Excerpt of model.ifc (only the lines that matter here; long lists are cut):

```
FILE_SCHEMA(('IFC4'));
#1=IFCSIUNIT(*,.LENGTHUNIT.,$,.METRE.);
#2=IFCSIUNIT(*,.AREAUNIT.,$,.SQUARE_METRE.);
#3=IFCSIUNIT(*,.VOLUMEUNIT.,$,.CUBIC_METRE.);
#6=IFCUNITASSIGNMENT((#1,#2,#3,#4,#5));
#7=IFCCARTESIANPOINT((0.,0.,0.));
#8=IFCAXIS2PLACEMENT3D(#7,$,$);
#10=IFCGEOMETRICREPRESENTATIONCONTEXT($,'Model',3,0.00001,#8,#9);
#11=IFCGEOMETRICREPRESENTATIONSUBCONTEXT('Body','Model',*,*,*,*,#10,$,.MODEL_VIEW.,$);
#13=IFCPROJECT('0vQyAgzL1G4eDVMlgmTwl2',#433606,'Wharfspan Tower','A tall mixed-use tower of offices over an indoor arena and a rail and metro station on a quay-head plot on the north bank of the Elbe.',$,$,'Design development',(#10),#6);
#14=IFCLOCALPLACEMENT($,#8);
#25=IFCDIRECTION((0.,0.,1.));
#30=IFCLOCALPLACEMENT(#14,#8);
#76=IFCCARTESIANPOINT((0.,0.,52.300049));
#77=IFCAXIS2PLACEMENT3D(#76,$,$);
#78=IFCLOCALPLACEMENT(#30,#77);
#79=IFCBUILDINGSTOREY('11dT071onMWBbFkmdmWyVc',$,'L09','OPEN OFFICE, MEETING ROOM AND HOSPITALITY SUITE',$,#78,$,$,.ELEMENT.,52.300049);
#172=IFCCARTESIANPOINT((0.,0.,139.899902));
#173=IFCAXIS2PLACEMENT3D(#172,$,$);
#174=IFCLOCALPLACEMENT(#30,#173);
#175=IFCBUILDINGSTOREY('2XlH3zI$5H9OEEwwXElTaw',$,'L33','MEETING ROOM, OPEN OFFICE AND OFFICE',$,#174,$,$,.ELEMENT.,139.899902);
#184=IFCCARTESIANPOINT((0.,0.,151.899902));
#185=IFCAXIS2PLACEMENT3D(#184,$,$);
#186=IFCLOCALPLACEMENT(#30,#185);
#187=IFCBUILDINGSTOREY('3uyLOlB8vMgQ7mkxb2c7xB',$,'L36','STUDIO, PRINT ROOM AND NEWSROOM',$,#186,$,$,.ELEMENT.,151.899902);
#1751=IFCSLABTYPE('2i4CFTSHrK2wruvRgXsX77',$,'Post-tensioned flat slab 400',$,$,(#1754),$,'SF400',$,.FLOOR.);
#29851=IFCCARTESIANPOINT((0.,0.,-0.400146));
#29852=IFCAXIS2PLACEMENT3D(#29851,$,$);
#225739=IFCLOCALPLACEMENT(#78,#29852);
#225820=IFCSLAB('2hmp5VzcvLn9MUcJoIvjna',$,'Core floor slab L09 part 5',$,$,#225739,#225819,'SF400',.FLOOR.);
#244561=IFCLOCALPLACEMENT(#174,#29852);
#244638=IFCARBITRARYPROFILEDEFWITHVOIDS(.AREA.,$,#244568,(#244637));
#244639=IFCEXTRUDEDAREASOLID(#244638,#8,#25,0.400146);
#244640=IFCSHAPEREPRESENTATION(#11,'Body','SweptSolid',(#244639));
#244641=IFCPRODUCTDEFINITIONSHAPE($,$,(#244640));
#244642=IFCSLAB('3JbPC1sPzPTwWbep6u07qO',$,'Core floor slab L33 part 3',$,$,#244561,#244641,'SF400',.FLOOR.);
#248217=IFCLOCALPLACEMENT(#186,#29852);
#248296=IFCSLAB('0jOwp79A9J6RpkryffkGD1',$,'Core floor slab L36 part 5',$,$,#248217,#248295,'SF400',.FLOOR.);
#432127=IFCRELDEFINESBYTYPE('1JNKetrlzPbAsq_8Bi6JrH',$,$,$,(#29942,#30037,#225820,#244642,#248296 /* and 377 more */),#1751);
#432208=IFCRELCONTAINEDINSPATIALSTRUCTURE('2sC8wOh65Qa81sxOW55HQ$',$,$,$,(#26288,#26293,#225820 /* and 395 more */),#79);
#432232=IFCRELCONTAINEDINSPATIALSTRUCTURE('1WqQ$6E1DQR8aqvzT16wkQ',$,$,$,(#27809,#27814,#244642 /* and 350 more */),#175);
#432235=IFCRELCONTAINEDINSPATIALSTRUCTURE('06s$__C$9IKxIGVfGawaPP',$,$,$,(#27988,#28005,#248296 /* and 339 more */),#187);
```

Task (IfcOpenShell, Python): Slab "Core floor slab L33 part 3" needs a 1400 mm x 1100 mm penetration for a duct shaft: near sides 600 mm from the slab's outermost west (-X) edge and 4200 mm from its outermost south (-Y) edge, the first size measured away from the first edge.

```python
import numpy as np
import ifcopenshell
import ifcopenshell.api.feature
import ifcopenshell.api.geometry
import ifcopenshell.api.root
import ifcopenshell.geom
import ifcopenshell.util.placement
import ifcopenshell.util.representation
import ifcopenshell.util.shape
import ifcopenshell.util.unit

model = ifcopenshell.open("model.ifc")
unit_scale = ifcopenshell.util.unit.calculate_unit_scale(model)
settings = ifcopenshell.geom.settings()


def volume(element):
    """Net volume in cubic metres, openings subtracted."""
    shape = ifcopenshell.geom.create_shape(settings, element)
    return ifcopenshell.util.shape.get_volume(shape.geometry)


slab = model.by_id(244642)
before = volume(slab)

# Extent in the slab's own axes, in metres. The edges named are its -X and -Y sides.
slab_shape = ifcopenshell.geom.create_shape(settings, slab)
vertices = ifcopenshell.util.shape.get_vertices(slab_shape.geometry)
x_min, y_min, bottom = vertices.min(axis=0)
top = vertices[:, 2].max()

opening = ifcopenshell.api.root.create_entity(model, ifc_class="IfcOpeningElement", name="Duct shaft opening", predefined_type="OPENING")
context = ifcopenshell.util.representation.get_context(model, "Model", "Body", "MODEL_VIEW")
width, depth = 1.4, 1.1
outline = [(0.0, 0.0), (width, 0.0), (width, depth), (0.0, depth), (0.0, 0.0)]
# Overshoot both faces by 50 mm so the cut is clean.
shape = ifcopenshell.api.geometry.add_slab_representation(
    model, context=context, depth=top - bottom + 0.1, polyline=outline
)
ifcopenshell.api.geometry.assign_representation(model, product=opening, representation=shape)

matrix = ifcopenshell.util.placement.get_local_placement(slab.ObjectPlacement)
matrix[:, 3] = matrix @ np.append(np.array([x_min + 0.6, y_min + 4.2, bottom - 0.05]) / unit_scale, 1.0)
ifcopenshell.api.geometry.edit_object_placement(model, product=opening, matrix=matrix, is_si=False)
ifcopenshell.api.feature.add_feature(model, feature=opening, element=slab)

after = volume(slab)

print(f"slab volume {before:.3f} -> {after:.3f} m3")

model.write("model_v2.ifc")
```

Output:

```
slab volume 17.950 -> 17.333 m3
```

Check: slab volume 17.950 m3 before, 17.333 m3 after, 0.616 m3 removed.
